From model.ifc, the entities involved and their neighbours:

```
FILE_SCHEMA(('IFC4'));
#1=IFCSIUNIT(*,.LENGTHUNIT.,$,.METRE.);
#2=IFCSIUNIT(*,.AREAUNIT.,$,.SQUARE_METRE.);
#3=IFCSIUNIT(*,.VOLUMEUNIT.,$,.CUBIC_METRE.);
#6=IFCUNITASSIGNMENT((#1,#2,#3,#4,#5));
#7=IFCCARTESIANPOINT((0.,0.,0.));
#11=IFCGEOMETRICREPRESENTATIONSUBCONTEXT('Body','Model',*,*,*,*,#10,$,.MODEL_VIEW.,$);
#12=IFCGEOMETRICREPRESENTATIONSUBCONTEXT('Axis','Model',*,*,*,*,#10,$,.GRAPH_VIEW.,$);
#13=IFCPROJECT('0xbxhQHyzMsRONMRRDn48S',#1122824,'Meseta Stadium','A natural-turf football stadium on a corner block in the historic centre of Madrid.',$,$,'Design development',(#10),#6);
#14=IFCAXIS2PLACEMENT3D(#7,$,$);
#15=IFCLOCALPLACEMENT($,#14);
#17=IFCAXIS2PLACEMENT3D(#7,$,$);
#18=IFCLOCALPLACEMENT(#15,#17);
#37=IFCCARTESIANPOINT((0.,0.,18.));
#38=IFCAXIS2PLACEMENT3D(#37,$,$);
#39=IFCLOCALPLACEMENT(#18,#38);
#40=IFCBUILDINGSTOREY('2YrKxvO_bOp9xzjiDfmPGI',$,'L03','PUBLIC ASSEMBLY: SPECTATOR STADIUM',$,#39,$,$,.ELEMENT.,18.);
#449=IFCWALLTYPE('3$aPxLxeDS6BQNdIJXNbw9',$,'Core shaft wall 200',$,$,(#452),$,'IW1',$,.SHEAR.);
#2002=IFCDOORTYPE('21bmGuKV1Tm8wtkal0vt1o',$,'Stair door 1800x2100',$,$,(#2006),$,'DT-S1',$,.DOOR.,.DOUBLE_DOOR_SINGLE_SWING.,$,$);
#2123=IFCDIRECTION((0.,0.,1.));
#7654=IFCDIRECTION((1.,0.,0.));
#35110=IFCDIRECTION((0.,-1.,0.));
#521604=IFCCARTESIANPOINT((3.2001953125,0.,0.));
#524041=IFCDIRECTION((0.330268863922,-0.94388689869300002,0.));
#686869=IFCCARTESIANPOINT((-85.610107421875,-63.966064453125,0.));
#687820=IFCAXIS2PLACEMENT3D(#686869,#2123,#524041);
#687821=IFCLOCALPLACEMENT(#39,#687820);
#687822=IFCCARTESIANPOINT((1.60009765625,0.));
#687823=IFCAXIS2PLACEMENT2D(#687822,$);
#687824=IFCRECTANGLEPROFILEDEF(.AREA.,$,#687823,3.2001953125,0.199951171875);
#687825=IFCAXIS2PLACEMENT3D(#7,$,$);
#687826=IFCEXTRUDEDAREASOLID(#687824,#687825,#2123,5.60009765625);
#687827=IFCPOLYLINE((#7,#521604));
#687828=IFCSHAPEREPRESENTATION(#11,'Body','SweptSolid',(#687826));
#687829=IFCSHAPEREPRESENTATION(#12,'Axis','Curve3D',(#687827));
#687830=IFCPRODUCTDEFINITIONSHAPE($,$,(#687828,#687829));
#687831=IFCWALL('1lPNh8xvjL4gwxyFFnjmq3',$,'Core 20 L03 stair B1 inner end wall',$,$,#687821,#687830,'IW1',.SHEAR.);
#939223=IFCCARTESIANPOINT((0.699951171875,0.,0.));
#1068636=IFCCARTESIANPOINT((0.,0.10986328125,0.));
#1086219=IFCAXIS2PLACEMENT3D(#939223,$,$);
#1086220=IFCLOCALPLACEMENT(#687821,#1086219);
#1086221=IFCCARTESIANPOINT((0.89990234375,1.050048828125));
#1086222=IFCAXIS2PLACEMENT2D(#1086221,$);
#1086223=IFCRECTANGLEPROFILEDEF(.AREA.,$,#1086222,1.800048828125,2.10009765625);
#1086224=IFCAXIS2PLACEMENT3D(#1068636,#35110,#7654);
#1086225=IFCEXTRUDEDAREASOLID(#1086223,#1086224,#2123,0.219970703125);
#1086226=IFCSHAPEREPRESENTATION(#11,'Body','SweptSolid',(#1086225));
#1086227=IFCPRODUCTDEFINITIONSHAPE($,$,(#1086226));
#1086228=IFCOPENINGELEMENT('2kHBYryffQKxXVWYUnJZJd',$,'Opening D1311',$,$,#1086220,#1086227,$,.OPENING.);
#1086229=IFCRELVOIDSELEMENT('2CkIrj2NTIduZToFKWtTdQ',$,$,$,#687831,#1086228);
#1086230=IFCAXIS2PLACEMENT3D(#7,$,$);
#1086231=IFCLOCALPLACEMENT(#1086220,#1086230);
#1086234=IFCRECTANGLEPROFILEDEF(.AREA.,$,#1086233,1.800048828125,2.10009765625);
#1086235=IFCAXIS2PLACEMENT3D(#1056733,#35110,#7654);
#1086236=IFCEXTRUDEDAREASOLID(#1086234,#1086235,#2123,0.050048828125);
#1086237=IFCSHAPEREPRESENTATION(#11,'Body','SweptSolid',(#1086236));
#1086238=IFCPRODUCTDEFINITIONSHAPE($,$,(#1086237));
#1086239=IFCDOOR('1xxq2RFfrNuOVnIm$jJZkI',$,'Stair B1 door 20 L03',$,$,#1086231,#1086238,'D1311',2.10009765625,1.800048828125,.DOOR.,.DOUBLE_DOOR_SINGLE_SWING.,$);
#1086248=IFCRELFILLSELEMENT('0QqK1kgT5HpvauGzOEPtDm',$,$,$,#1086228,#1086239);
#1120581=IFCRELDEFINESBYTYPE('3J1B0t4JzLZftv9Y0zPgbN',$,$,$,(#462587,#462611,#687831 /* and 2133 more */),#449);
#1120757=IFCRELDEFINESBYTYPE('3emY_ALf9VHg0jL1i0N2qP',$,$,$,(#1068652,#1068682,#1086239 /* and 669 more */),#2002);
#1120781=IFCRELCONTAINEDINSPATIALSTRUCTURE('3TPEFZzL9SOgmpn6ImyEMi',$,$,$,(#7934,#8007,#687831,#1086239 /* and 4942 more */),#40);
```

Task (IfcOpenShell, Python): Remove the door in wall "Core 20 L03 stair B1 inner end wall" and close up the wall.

```python
import ifcopenshell
import ifcopenshell.api.feature
import ifcopenshell.api.root
import ifcopenshell.geom
import ifcopenshell.util.shape

model = ifcopenshell.open("model.ifc")
settings = ifcopenshell.geom.settings()


def volume(element):
    """Net volume in cubic metres, openings subtracted."""
    shape = ifcopenshell.geom.create_shape(settings, element)
    return ifcopenshell.util.shape.get_volume(shape.geometry)


door = model.by_guid("1xxq2RFfrNuOVnIm$jJZkI")
opening = door.FillsVoids[0].RelatingOpeningElement
wall = opening.VoidsElements[0].RelatingBuildingElement
before = volume(wall)

ifcopenshell.api.root.remove_product(model, product=door)
ifcopenshell.api.feature.remove_feature(model, feature=opening)

after = volume(wall)

print(f"wall volume {before:.3f} -> {after:.3f} m3")

model.write("model_edited.ifc")
```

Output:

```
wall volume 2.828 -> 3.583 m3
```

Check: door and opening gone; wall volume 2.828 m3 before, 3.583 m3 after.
